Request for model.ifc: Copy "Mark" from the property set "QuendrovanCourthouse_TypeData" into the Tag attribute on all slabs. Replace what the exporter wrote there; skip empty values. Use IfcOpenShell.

First a look at what the model holds.

```python
import ifcopenshell
import ifcopenshell.util.element

model = ifcopenshell.open("model.ifc")
print(model.schema)
slabs = model.by_type("IfcSlab")
print(len(slabs), "slabs")
for e in slabs[:8]:
    source = ifcopenshell.util.element.get_pset(e, "QuendrovanCourthouse_TypeData", "Mark")
    target = e.Tag
    print(e.id(), repr(source), repr(target), sep=" | ")
```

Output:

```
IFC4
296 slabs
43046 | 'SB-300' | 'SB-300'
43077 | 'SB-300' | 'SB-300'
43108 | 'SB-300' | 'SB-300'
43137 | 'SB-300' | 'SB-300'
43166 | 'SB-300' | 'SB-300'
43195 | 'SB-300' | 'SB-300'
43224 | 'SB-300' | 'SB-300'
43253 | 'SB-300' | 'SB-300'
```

```python
import ifcopenshell
import ifcopenshell.util.element

model = ifcopenshell.open("model.ifc")

count = 0
for e in model.by_type("IfcSlab"):
    value = ifcopenshell.util.element.get_pset(e, "QuendrovanCourthouse_TypeData", "Mark")
    current = e.Tag
    if not value or not value.strip() or current == value:
        continue
    e.Tag = value
    count += 1

print(count, "slabs updated")

model.write("model_updated.ifc")
```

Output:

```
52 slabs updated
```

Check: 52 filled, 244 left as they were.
